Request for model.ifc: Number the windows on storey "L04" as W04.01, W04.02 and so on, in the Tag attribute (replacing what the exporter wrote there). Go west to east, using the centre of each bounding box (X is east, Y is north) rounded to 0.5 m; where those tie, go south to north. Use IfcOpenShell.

First a look at what the model holds.

```python
import ifcopenshell
import ifcopenshell.util.element
import ifcopenshell.util.placement

model = ifcopenshell.open("model.ifc")
print(model.schema)
storey = next(s for s in model.by_type("IfcBuildingStorey") if s.Name == "L04")
windows = [e for e in ifcopenshell.util.element.get_decomposition(storey) if e.is_a("IfcWindow")]
for e in sorted(windows, key=lambda e: e.id()):
    origin = ifcopenshell.util.placement.get_local_placement(e.ObjectPlacement)[:3, 3]
    print(e.id(), e.Tag, e.Name, origin.round(2) + 0.0, sep=" | ")
```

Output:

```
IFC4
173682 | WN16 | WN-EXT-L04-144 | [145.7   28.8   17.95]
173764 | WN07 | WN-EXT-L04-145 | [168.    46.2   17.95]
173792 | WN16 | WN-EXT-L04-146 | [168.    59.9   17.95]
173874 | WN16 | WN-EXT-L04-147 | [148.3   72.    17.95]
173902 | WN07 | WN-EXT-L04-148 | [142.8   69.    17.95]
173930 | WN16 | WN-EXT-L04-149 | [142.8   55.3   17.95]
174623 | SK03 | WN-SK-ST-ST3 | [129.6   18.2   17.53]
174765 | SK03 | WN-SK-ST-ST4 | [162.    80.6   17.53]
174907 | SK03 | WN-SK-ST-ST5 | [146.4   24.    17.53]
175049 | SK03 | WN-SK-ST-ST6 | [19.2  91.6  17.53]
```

```python
import ifcopenshell
import ifcopenshell.geom
import ifcopenshell.util.element
import ifcopenshell.util.shape

model = ifcopenshell.open("model.ifc")
settings = ifcopenshell.geom.settings()
settings.set("use-world-coords", True)


def centre(element):
    shape = ifcopenshell.geom.create_shape(settings, element)
    return ifcopenshell.util.shape.get_bbox_centroid(shape.geometry)


storey = next(s for s in model.by_type("IfcBuildingStorey") if s.Name == "L04")
windows = [e for e in ifcopenshell.util.element.get_decomposition(storey) if e.is_a("IfcWindow")]

# Insertion points can sit at a corner or the storey origin, so sort by the geometry (in metres).
centres = {e: centre(e) for e in windows}
windows.sort(key=lambda e: (round(centres[e][0] / 0.5), centres[e][1]))

for i, e in enumerate(windows, start=1):
    number = f"W04.{i:02d}"
    e.Tag = number
    print(e.id(), number)

model.write("model_edited.ifc")
```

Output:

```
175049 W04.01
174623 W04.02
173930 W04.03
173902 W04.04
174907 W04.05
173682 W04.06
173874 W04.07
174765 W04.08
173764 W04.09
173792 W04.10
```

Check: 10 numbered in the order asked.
